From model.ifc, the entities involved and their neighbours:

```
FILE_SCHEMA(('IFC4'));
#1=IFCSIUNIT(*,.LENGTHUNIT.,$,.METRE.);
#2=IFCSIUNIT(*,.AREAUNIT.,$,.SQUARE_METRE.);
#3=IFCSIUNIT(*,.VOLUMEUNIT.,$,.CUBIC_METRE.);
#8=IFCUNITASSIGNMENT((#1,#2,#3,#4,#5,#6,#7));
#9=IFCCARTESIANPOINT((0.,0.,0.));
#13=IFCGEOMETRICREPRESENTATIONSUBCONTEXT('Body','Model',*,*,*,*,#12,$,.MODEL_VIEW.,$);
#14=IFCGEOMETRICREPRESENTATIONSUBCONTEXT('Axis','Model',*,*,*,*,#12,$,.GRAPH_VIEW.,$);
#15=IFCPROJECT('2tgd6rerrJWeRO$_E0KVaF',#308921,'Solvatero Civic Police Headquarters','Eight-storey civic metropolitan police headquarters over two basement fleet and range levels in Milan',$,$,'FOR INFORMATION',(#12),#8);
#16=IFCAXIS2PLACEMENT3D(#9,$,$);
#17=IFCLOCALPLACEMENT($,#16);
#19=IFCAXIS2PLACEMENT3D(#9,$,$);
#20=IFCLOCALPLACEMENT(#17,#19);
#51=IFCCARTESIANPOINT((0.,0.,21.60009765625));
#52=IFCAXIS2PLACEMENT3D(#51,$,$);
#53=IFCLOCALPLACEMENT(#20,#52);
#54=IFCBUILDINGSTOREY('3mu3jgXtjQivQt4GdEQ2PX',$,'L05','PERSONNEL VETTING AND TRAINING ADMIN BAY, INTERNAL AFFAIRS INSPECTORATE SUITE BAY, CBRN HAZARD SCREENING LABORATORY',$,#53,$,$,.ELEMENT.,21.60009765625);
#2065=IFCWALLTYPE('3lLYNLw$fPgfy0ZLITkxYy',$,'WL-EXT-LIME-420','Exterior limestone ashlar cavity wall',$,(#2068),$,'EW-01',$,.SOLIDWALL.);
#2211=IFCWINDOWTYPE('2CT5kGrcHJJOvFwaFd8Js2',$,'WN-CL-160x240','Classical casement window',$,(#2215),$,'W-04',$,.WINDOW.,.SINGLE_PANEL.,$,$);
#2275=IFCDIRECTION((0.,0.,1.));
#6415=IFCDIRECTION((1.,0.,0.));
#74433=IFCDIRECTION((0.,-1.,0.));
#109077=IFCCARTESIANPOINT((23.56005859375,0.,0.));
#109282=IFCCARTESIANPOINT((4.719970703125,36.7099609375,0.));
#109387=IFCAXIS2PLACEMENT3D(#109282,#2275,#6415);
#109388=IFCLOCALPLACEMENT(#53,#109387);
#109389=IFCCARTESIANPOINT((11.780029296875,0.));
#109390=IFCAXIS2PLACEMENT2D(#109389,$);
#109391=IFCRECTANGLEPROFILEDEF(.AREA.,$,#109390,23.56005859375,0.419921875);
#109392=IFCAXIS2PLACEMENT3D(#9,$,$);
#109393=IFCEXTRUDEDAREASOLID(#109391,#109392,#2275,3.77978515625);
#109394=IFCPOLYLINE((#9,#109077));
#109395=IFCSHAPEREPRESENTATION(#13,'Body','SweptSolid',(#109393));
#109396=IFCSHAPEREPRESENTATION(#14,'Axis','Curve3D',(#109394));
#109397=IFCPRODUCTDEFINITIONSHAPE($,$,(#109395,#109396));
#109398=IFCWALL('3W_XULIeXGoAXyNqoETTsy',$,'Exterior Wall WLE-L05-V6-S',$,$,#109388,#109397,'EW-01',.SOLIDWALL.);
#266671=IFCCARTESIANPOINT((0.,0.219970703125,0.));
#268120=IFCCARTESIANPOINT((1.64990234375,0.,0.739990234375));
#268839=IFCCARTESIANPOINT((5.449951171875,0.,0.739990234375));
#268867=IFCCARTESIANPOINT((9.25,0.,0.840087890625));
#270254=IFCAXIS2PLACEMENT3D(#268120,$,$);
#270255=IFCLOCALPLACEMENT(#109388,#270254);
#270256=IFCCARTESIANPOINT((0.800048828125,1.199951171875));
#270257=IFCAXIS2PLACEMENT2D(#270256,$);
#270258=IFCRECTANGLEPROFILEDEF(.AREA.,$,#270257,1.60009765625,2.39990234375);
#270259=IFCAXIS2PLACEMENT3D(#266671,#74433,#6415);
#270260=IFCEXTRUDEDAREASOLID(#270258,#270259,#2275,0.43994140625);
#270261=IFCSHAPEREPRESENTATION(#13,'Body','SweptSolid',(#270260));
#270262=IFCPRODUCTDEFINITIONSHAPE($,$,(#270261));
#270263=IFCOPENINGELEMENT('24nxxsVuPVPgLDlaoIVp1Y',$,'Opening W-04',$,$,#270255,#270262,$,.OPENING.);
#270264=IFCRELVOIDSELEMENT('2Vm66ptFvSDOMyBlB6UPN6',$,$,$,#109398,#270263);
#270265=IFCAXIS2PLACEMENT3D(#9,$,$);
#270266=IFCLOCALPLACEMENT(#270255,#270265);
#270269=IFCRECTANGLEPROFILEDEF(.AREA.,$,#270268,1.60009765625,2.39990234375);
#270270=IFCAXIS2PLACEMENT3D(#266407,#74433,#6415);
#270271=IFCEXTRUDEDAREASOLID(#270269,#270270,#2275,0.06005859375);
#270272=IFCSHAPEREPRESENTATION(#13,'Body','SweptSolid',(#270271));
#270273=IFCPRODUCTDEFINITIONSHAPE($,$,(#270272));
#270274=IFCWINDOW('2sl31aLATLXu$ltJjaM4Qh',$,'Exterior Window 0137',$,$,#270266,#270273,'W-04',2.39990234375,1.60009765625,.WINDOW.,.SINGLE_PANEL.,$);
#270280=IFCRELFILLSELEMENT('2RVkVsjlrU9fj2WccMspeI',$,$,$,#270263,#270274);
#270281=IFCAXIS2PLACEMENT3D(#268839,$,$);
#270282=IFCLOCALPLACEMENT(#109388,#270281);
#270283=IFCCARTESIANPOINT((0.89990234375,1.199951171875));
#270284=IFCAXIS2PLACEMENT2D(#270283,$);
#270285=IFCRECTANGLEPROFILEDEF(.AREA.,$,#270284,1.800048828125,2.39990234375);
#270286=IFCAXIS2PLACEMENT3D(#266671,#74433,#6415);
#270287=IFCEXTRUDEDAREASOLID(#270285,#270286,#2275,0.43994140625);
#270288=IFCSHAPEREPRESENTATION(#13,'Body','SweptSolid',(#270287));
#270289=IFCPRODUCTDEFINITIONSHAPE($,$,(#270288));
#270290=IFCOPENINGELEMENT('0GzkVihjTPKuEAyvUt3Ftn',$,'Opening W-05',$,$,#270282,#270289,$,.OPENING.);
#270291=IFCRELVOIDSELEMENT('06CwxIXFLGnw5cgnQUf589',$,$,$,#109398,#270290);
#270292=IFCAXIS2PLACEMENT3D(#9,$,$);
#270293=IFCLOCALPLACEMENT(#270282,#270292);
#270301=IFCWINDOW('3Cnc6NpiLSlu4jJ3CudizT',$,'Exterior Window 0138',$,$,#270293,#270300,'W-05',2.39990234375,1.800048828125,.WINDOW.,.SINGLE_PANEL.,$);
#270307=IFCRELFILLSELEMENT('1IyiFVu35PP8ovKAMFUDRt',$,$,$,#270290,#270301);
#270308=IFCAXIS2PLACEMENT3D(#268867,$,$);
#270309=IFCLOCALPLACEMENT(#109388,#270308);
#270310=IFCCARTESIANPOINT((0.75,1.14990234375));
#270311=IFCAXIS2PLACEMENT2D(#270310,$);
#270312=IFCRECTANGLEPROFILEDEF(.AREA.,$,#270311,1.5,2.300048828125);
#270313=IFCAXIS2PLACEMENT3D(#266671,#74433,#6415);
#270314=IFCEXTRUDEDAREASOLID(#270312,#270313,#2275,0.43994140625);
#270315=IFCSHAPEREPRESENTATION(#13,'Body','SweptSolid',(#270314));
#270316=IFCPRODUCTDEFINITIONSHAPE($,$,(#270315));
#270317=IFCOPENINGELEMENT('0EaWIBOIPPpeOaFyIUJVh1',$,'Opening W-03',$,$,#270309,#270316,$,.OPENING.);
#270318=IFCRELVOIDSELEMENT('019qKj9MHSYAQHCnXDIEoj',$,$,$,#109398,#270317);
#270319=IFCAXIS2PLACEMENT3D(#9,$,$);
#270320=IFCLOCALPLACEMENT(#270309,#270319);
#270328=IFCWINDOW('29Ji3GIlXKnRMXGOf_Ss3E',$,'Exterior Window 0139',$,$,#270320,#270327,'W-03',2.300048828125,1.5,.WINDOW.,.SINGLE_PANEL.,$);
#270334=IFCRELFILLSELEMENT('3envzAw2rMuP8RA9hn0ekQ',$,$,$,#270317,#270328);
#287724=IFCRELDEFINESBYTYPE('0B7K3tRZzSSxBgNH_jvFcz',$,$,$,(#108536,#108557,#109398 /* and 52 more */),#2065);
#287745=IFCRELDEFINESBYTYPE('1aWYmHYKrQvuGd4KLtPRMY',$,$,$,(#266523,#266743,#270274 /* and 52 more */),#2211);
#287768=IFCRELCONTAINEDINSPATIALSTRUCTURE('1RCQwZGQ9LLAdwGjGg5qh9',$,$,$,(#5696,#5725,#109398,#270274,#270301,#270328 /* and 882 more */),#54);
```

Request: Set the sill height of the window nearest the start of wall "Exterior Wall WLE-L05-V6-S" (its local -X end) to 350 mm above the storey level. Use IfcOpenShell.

```python
import numpy as np
import ifcopenshell
import ifcopenshell.api.geometry
import ifcopenshell.geom
import ifcopenshell.util.element
import ifcopenshell.util.placement
import ifcopenshell.util.shape
import ifcopenshell.util.unit

model = ifcopenshell.open("model.ifc")
unit_scale = ifcopenshell.util.unit.calculate_unit_scale(model)

window = model.by_id(270274)
opening = window.FillsVoids[0].RelatingOpeningElement
storey = ifcopenshell.util.element.get_container(window, ifc_class="IfcBuildingStorey")
level = ifcopenshell.util.placement.get_local_placement(storey.ObjectPlacement)[2, 3]

# The opening's origin need not be at the sill, so measure its lowest point.
shape = ifcopenshell.geom.create_shape(ifcopenshell.geom.settings(), opening)
bottom = ifcopenshell.util.shape.get_shape_bottom_elevation(shape, shape.geometry) / unit_scale
dz = level + 0.35 - bottom

shift = np.array([0.0, 0.0, dz])
# The window is placed relative to its opening, so it follows when the opening moves.
matrix = ifcopenshell.util.placement.get_local_placement(opening.ObjectPlacement)
matrix[:3, 3] += shift
ifcopenshell.api.geometry.edit_object_placement(
    model, product=opening, matrix=matrix, is_si=False, should_transform_children=True
)

print(f"moved by {dz * unit_scale:+.3f} m")

model.write("model_edited.ifc")
```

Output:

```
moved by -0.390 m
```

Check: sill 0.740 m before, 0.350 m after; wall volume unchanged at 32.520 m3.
